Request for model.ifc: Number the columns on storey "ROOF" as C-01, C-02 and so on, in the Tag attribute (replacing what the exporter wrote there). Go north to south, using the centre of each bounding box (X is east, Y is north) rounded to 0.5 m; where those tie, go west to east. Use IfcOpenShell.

First a look at what the model holds.

```python
import ifcopenshell
import ifcopenshell.util.element
import ifcopenshell.util.placement

model = ifcopenshell.open("model.ifc")
print(model.schema)
storey = next(s for s in model.by_type("IfcBuildingStorey") if s.Name == "ROOF")
columns = [e for e in ifcopenshell.util.element.get_decomposition(storey) if e.is_a("IfcColumn")]
for e in sorted(columns, key=lambda e: e.id()):
    origin = ifcopenshell.util.placement.get_local_placement(e.ObjectPlacement)[:3, 3]
    print(e.id(), e.Tag, e.Name, origin.round(2) + 0.0, sep=" | ")
```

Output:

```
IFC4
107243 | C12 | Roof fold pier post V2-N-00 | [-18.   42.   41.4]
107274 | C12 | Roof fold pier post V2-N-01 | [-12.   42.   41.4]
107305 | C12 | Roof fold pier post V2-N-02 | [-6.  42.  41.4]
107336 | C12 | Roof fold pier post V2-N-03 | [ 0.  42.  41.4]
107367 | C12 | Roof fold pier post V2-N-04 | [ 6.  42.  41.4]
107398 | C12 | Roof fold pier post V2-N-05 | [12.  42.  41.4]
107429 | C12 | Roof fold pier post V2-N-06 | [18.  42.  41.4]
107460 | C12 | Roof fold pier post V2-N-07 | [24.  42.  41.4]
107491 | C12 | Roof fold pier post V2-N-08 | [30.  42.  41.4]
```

```python
import ifcopenshell
import ifcopenshell.geom
import ifcopenshell.util.element
import ifcopenshell.util.shape

model = ifcopenshell.open("model.ifc")
settings = ifcopenshell.geom.settings()
settings.set("use-world-coords", True)


def centre(element):
    shape = ifcopenshell.geom.create_shape(settings, element)
    return ifcopenshell.util.shape.get_bbox_centroid(shape.geometry)


storey = next(s for s in model.by_type("IfcBuildingStorey") if s.Name == "ROOF")
columns = [e for e in ifcopenshell.util.element.get_decomposition(storey) if e.is_a("IfcColumn")]

# Insertion points can sit at a corner or the storey origin, so sort by the geometry (in metres).
centres = {e: centre(e) for e in columns}
columns.sort(key=lambda e: (-round(centres[e][1] / 0.5), centres[e][0]))

for i, e in enumerate(columns, start=1):
    number = f"C-{i:02d}"
    e.Tag = number
    print(e.id(), number)

model.write("model-out.ifc")
```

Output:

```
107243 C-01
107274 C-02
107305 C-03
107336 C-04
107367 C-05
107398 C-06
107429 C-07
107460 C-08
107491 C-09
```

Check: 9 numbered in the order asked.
